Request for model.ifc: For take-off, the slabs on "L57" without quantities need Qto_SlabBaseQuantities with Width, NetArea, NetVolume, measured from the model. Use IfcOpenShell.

First a look at what the model holds.

```python
import ifcopenshell
import ifcopenshell.util.element
import ifcopenshell.util.unit

model = ifcopenshell.open("model.ifc")
print(model.schema)
for unit_type in ("LENGTHUNIT", "AREAUNIT", "VOLUMEUNIT"):
    print(unit_type, ifcopenshell.util.unit.calculate_unit_scale(model, unit_type))
storey = next(s for s in model.by_type("IfcBuildingStorey") if s.Name == "L57")
slabs = [e for e in ifcopenshell.util.element.get_decomposition(storey) if e.is_a("IfcSlab")]
for e in sorted(slabs, key=lambda e: e.id()):
    print(e.id(), e.is_a(), e.Name, list(ifcopenshell.util.element.get_psets(e, qtos_only=True)), sep=" | ")
```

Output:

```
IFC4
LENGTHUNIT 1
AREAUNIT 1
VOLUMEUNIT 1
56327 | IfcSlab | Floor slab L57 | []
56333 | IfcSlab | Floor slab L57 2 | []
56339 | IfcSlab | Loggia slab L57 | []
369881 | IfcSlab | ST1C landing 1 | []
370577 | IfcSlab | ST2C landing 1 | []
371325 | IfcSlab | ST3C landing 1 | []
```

```python
import ifcopenshell
import ifcopenshell.api.pset
import ifcopenshell.geom
import ifcopenshell.util.element
import ifcopenshell.util.shape
import ifcopenshell.util.unit

model = ifcopenshell.open("model.ifc")
unit_scale = ifcopenshell.util.unit.calculate_unit_scale(model)
area_scale = ifcopenshell.util.unit.calculate_unit_scale(model, "AREAUNIT")
volume_scale = ifcopenshell.util.unit.calculate_unit_scale(model, "VOLUMEUNIT")
settings = ifcopenshell.geom.settings()

storey = next(s for s in model.by_type("IfcBuildingStorey") if s.Name == "L57")
slabs = [e for e in ifcopenshell.util.element.get_decomposition(storey) if e.is_a("IfcSlab")]

for e in sorted(slabs, key=lambda e: e.id()):
    if ifcopenshell.util.element.get_psets(e, qtos_only=True, should_inherit=False):
        continue
    # Geometry comes back in metres, in the element's own axes.
    shape = ifcopenshell.geom.create_shape(settings, e)
    values = {
        "Width": ifcopenshell.util.shape.get_z(shape.geometry) / unit_scale,
        "NetArea": ifcopenshell.util.shape.get_footprint_area(shape.geometry) / area_scale,
        "NetVolume": ifcopenshell.util.shape.get_volume(shape.geometry) / volume_scale,
    }
    qto = ifcopenshell.api.pset.add_qto(model, product=e, name="Qto_SlabBaseQuantities")
    ifcopenshell.api.pset.edit_qto(model, qto=qto, properties=values)
    print(e.id(), {k: round(v, 3) for k, v in values.items()})

model.write("model_edited.ifc")
```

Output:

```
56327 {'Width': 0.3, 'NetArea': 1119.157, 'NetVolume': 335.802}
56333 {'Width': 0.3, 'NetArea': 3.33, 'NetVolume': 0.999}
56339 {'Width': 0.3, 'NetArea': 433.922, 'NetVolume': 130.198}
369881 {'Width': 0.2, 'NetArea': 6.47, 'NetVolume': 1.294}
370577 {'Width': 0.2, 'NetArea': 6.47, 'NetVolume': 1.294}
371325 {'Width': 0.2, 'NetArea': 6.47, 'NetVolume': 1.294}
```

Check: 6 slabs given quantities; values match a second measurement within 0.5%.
